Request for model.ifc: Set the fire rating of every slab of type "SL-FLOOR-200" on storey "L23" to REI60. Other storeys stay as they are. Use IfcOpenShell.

First a look at what the model holds.

```python
import ifcopenshell
import ifcopenshell.util.element

model = ifcopenshell.open("model.ifc")
print(model.schema)
storey = next(s for s in model.by_type("IfcBuildingStorey") if s.Name == "L23")
slabs = [e for e in ifcopenshell.util.element.get_decomposition(storey) if e.is_a("IfcSlab")]
seen = {}
for e in slabs:
    element_type = ifcopenshell.util.element.get_type(e)
    key = (element_type.Name if element_type != e and element_type else None, ifcopenshell.util.element.get_pset(e, "Pset_SlabCommon", "FireRating"))
    seen[key] = seen.get(key, 0) + 1
for (name, value), count in sorted(seen.items(), key=str):
    print(count, "x", name, "|", value)
```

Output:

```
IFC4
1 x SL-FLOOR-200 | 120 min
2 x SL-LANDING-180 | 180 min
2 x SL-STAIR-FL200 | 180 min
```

```python
import ifcopenshell
import ifcopenshell.api.pset
import ifcopenshell.util.element

model = ifcopenshell.open("model.ifc")

storey = next(s for s in model.by_type("IfcBuildingStorey") if s.Name == "L23")
slabs = [e for e in ifcopenshell.util.element.get_decomposition(storey) if e.is_a("IfcSlab")]

count = 0
for e in slabs:
    element_type = ifcopenshell.util.element.get_type(e)
    if element_type in (None, e) or element_type.Name != "SL-FLOOR-200":
        continue
    found = ifcopenshell.util.element.get_pset(e, "Pset_SlabCommon", should_inherit=False)
    if found:
        pset = model.by_id(found["id"])
        if len(ifcopenshell.util.element.get_elements_by_pset(pset)) > 1:
            pset = ifcopenshell.api.pset.unshare_pset(model, products=[e], pset=pset)[0]
    else:
        pset = ifcopenshell.api.pset.add_pset(model, product=e, name="Pset_SlabCommon")
    ifcopenshell.api.pset.edit_pset(model, pset=pset, properties={"FireRating": "REI60"})
    count += 1

print(count, "slabs updated")

model.write("model_edited.ifc")
```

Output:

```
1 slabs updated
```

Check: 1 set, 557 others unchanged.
